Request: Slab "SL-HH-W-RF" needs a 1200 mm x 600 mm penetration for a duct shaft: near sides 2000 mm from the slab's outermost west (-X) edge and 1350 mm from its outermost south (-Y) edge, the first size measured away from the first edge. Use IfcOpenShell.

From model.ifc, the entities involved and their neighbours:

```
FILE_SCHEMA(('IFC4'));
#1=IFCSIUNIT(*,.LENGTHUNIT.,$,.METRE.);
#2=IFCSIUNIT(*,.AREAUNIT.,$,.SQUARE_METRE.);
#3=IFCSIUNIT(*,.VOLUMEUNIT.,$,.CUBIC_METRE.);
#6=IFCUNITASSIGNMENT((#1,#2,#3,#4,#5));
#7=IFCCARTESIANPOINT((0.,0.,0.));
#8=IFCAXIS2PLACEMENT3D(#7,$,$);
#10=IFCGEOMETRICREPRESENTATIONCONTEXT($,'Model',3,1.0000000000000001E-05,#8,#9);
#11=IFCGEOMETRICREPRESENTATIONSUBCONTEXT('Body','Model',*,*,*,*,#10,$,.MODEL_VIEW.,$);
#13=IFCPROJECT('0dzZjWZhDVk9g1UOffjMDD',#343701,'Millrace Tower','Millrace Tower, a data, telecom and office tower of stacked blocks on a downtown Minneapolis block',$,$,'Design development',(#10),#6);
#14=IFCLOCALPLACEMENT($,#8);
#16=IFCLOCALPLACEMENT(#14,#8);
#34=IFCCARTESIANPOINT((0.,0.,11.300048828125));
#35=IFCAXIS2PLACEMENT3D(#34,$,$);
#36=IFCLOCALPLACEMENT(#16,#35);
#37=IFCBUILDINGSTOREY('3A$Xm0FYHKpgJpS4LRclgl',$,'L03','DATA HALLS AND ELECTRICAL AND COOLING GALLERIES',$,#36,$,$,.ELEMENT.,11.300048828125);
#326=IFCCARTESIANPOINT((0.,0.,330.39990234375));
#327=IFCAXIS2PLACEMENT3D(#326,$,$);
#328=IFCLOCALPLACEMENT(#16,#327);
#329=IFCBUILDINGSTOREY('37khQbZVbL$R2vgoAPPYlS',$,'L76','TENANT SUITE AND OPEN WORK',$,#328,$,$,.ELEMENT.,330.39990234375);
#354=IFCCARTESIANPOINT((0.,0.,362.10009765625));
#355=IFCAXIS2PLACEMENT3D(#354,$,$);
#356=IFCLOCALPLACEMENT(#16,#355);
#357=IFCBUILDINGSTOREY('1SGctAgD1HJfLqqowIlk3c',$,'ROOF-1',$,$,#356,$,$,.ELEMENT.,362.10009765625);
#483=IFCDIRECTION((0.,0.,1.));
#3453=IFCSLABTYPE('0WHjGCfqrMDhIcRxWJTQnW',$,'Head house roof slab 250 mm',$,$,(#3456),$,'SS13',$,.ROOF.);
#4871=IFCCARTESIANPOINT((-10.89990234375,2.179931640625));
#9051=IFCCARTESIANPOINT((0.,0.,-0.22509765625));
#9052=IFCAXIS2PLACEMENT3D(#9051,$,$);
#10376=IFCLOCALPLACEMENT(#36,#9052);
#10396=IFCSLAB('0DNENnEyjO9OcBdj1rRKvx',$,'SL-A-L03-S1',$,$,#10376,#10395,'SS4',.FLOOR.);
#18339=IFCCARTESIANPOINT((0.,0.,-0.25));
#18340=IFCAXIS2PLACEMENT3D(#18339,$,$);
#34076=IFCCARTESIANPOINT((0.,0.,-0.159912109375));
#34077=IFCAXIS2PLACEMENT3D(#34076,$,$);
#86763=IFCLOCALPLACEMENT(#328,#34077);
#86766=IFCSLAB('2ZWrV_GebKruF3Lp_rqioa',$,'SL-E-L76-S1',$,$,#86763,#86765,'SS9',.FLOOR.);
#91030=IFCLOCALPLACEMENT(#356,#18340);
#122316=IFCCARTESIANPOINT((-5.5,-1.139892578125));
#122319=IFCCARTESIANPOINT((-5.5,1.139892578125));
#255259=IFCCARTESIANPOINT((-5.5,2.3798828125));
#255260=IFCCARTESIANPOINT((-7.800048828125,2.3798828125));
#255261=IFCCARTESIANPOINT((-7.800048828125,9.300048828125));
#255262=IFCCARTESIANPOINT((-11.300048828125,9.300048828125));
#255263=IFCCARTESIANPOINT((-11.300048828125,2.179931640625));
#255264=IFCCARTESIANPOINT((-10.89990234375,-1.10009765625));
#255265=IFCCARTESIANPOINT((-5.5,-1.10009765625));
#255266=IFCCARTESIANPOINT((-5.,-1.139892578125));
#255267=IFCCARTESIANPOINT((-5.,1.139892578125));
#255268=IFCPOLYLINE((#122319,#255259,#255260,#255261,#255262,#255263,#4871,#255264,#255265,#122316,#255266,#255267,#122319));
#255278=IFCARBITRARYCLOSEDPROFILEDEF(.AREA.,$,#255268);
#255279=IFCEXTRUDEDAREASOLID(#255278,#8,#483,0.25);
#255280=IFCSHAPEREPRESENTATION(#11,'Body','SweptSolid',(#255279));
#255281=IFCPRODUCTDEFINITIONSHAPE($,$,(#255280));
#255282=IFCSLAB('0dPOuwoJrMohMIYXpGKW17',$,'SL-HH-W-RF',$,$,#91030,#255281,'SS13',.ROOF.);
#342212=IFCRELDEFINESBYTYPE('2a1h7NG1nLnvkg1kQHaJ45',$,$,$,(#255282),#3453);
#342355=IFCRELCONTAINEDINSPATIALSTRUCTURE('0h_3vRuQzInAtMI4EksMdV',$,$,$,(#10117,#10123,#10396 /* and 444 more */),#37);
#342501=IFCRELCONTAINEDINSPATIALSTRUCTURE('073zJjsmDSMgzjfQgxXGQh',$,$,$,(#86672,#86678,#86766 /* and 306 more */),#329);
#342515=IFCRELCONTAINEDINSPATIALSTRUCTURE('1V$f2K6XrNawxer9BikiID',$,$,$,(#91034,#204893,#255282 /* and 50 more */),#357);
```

```python
import numpy as np
import ifcopenshell
import ifcopenshell.api.feature
import ifcopenshell.api.geometry
import ifcopenshell.api.root
import ifcopenshell.geom
import ifcopenshell.util.placement
import ifcopenshell.util.representation
import ifcopenshell.util.shape
import ifcopenshell.util.unit

model = ifcopenshell.open("model.ifc")
unit_scale = ifcopenshell.util.unit.calculate_unit_scale(model)
settings = ifcopenshell.geom.settings()


def volume(element):
    """Net volume in cubic metres, openings subtracted."""
    shape = ifcopenshell.geom.create_shape(settings, element)
    return ifcopenshell.util.shape.get_volume(shape.geometry)


slab = model.by_guid("0dPOuwoJrMohMIYXpGKW17")
before = volume(slab)

# Extent in the slab's own axes, in metres. The edges named are its -X and -Y sides.
slab_shape = ifcopenshell.geom.create_shape(settings, slab)
vertices = ifcopenshell.util.shape.get_vertices(slab_shape.geometry)
x_min, y_min, bottom = vertices.min(axis=0)
top = vertices[:, 2].max()

opening = ifcopenshell.api.root.create_entity(model, ifc_class="IfcOpeningElement", name="Duct shaft opening", predefined_type="OPENING")
context = ifcopenshell.util.representation.get_context(model, "Model", "Body", "MODEL_VIEW")
width, depth = 1.2, 0.6
outline = [(0.0, 0.0), (width, 0.0), (width, depth), (0.0, depth), (0.0, 0.0)]
# Overshoot both faces by 50 mm so the cut is clean.
shape = ifcopenshell.api.geometry.add_slab_representation(
    model, context=context, depth=top - bottom + 0.1, polyline=outline
)
ifcopenshell.api.geometry.assign_representation(model, product=opening, representation=shape)

matrix = ifcopenshell.util.placement.get_local_placement(slab.ObjectPlacement)
matrix[:, 3] = matrix @ np.append(np.array([x_min + 2, y_min + 1.35, bottom - 0.05]) / unit_scale, 1.0)
ifcopenshell.api.geometry.edit_object_placement(model, product=opening, matrix=matrix, is_si=False)
ifcopenshell.api.feature.add_feature(model, feature=opening, element=slab)

after = volume(slab)

print(f"slab volume {before:.3f} -> {after:.3f} m3")

model.write("model_v2.ifc")
```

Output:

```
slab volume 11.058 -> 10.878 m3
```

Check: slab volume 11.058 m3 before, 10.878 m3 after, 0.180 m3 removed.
